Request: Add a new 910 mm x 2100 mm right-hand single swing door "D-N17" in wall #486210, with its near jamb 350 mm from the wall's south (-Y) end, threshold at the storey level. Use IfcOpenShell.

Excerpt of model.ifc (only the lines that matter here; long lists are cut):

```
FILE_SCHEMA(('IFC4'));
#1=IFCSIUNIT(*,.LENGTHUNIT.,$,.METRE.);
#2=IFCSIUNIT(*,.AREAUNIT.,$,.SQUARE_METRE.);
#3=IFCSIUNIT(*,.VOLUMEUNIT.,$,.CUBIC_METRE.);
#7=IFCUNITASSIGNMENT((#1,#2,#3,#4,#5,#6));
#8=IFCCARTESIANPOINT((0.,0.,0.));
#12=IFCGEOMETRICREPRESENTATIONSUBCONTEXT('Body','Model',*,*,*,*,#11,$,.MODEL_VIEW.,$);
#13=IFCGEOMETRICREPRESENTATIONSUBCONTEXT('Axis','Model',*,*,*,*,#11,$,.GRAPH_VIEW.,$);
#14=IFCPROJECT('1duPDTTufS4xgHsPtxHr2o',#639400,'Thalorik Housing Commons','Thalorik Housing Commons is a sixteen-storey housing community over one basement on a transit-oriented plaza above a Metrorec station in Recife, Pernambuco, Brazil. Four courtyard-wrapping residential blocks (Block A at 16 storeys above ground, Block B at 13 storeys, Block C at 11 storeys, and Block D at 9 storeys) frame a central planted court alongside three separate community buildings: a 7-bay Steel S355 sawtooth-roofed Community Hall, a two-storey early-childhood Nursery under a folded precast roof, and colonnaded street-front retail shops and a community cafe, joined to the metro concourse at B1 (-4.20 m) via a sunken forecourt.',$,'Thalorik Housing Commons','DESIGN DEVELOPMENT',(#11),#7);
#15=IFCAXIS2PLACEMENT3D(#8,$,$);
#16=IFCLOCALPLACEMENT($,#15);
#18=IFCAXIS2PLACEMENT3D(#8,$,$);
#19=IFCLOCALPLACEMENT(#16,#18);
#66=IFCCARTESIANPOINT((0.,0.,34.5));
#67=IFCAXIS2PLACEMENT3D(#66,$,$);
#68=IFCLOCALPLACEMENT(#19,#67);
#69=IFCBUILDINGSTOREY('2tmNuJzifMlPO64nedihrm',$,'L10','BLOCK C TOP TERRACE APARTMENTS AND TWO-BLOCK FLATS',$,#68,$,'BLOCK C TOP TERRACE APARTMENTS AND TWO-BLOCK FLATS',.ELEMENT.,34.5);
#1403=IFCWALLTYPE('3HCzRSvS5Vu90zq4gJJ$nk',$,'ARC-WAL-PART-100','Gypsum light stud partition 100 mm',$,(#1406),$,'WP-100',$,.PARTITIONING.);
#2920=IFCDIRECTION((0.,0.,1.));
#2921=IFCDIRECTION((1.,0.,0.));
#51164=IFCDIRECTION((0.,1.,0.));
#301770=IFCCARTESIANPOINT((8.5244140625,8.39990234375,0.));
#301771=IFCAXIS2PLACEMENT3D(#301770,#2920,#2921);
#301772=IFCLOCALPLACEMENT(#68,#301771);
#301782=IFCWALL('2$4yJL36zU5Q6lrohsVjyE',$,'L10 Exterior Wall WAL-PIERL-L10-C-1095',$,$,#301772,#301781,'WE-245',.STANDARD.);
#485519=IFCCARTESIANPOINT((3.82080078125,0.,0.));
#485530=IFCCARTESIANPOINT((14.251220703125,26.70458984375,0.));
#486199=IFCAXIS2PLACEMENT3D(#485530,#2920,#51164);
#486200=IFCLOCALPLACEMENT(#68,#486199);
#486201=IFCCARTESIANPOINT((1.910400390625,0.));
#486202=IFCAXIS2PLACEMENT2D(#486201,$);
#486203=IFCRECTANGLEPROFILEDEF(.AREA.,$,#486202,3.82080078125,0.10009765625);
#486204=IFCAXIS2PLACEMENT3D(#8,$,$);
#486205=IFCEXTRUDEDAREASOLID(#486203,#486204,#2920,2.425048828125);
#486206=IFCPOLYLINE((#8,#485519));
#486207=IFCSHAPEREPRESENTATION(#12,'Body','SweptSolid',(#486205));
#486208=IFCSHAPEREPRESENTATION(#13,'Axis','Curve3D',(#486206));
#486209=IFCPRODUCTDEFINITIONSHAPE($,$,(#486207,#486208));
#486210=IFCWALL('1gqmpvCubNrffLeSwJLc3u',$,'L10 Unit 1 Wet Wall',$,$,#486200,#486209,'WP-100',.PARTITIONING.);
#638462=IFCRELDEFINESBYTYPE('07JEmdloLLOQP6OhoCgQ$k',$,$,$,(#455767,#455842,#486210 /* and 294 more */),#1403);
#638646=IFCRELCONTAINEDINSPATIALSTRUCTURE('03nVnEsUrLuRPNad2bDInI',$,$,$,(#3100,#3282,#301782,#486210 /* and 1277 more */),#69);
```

```python
import numpy as np
import ifcopenshell
import ifcopenshell.api.feature
import ifcopenshell.api.geometry
import ifcopenshell.api.root
import ifcopenshell.api.spatial
import ifcopenshell.geom
import ifcopenshell.util.element
import ifcopenshell.util.placement
import ifcopenshell.util.representation
import ifcopenshell.util.shape
import ifcopenshell.util.unit

model = ifcopenshell.open("model.ifc")
unit_scale = ifcopenshell.util.unit.calculate_unit_scale(model)
settings = ifcopenshell.geom.settings()


def volume(element):
    """Net volume in cubic metres, openings subtracted."""
    shape = ifcopenshell.geom.create_shape(settings, element)
    return ifcopenshell.util.shape.get_volume(shape.geometry)


wall = model.by_guid("1gqmpvCubNrffLeSwJLc3u")
storey = ifcopenshell.util.element.get_container(wall, ifc_class="IfcBuildingStorey")
context = ifcopenshell.util.representation.get_context(model, "Model", "Body", "MODEL_VIEW")
before = volume(wall)

width, height, from_end, sill = 0.91, 2.1, 0.35, 0.0  # metres

# The wall runs along its own X axis, and the end named is its -X end.
wall_shape = ifcopenshell.geom.create_shape(settings, wall)
x, y, z = ifcopenshell.util.shape.get_vertices(wall_shape.geometry).T
start = x.min() + from_end
face, thickness = float(y.min()), float(y.max() - y.min())
wall_matrix = ifcopenshell.util.placement.get_local_placement(wall.ObjectPlacement)
level = ifcopenshell.util.placement.get_local_placement(storey.ObjectPlacement)[2, 3]


def in_wall(x, y):
    """Placement at x, y metres in the wall's axes, at sill height."""
    matrix = wall_matrix.copy()
    matrix[:, 3] = wall_matrix @ np.array([x / unit_scale, y / unit_scale, 0.0, 1.0])
    matrix[2, 3] = level + sill / unit_scale
    return matrix


# Opening: a box that overshoots both wall faces by 50 mm.
opening = ifcopenshell.api.root.create_entity(model, ifc_class="IfcOpeningElement", predefined_type="OPENING")
box = ifcopenshell.api.geometry.add_wall_representation(
    model, context=context, length=width, height=height, thickness=thickness + 0.1
)
ifcopenshell.api.geometry.assign_representation(model, product=opening, representation=box)
ifcopenshell.api.geometry.edit_object_placement(model, product=opening, matrix=in_wall(start, face - 0.05), is_si=False)
ifcopenshell.api.feature.add_feature(model, feature=opening, element=wall)

door = ifcopenshell.api.root.create_entity(model, ifc_class="IfcDoor", name="D-N17", predefined_type="DOOR")
door.OverallWidth, door.OverallHeight = width / unit_scale, height / unit_scale
door.OperationType = "SINGLE_SWING_RIGHT"
body = ifcopenshell.api.geometry.add_door_representation(
    model,
    context=context,
    overall_width=door.OverallWidth,
    overall_height=door.OverallHeight,
    operation_type="SINGLE_SWING_RIGHT",
    lining_properties={"LiningDepth": thickness / unit_scale, "ThresholdDepth": thickness / unit_scale},
)
ifcopenshell.api.geometry.assign_representation(model, product=door, representation=body)
ifcopenshell.api.spatial.assign_container(model, products=[door], relating_structure=storey)
ifcopenshell.api.feature.add_filling(model, opening=opening, element=door)

# The lining spans the wall, so the door starts at the wall face.
ifcopenshell.api.geometry.edit_object_placement(model, product=door, matrix=in_wall(start, face), is_si=False)

after = volume(wall)

print(f"wall volume {before:.3f} -> {after:.3f} m3")

model.write("model_edited.ifc")
```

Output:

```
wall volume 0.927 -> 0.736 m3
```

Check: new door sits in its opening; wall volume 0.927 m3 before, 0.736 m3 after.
